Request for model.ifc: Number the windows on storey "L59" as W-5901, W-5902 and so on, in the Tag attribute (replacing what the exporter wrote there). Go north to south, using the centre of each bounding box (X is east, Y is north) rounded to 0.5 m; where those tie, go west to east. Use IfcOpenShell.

First a look at what the model holds.

```python
import ifcopenshell
import ifcopenshell.util.element
import ifcopenshell.util.placement

model = ifcopenshell.open("model.ifc")
print(model.schema)
storey = next(s for s in model.by_type("IfcBuildingStorey") if s.Name == "L59")
windows = [e for e in ifcopenshell.util.element.get_decomposition(storey) if e.is_a("IfcWindow")]
for e in sorted(windows, key=lambda e: e.id()):
    origin = ifcopenshell.util.placement.get_local_placement(e.ObjectPlacement)[:3, 3]
    print(e.id(), e.Tag, e.Name, origin.round(2) + 0.0, sep=" | ")
```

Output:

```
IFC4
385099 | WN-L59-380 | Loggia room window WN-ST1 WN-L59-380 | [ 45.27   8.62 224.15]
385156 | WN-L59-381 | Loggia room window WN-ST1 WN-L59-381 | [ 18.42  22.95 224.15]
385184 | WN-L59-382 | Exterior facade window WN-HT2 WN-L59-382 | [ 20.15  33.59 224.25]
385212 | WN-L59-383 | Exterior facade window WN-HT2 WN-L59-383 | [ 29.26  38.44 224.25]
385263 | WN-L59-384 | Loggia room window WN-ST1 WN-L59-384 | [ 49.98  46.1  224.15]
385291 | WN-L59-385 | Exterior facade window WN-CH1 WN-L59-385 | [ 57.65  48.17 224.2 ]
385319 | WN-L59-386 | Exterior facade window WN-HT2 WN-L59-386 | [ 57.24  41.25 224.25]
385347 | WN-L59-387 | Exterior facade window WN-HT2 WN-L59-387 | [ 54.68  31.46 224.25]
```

```python
import ifcopenshell
import ifcopenshell.geom
import ifcopenshell.util.element
import ifcopenshell.util.shape

model = ifcopenshell.open("model.ifc")
settings = ifcopenshell.geom.settings()
settings.set("use-world-coords", True)


def centre(element):
    shape = ifcopenshell.geom.create_shape(settings, element)
    return ifcopenshell.util.shape.get_bbox_centroid(shape.geometry)


storey = next(s for s in model.by_type("IfcBuildingStorey") if s.Name == "L59")
windows = [e for e in ifcopenshell.util.element.get_decomposition(storey) if e.is_a("IfcWindow")]

# Insertion points can sit at a corner or the storey origin, so sort by the geometry (in metres).
centres = {e: centre(e) for e in windows}
windows.sort(key=lambda e: (-round(centres[e][1] / 0.5), centres[e][0]))

for i, e in enumerate(windows, start=1):
    number = f"W-59{i:02d}"
    e.Tag = number
    print(e.id(), number)

model.write("model_updated.ifc")
```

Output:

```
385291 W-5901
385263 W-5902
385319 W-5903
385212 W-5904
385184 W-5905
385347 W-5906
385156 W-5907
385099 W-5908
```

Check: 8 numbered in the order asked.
